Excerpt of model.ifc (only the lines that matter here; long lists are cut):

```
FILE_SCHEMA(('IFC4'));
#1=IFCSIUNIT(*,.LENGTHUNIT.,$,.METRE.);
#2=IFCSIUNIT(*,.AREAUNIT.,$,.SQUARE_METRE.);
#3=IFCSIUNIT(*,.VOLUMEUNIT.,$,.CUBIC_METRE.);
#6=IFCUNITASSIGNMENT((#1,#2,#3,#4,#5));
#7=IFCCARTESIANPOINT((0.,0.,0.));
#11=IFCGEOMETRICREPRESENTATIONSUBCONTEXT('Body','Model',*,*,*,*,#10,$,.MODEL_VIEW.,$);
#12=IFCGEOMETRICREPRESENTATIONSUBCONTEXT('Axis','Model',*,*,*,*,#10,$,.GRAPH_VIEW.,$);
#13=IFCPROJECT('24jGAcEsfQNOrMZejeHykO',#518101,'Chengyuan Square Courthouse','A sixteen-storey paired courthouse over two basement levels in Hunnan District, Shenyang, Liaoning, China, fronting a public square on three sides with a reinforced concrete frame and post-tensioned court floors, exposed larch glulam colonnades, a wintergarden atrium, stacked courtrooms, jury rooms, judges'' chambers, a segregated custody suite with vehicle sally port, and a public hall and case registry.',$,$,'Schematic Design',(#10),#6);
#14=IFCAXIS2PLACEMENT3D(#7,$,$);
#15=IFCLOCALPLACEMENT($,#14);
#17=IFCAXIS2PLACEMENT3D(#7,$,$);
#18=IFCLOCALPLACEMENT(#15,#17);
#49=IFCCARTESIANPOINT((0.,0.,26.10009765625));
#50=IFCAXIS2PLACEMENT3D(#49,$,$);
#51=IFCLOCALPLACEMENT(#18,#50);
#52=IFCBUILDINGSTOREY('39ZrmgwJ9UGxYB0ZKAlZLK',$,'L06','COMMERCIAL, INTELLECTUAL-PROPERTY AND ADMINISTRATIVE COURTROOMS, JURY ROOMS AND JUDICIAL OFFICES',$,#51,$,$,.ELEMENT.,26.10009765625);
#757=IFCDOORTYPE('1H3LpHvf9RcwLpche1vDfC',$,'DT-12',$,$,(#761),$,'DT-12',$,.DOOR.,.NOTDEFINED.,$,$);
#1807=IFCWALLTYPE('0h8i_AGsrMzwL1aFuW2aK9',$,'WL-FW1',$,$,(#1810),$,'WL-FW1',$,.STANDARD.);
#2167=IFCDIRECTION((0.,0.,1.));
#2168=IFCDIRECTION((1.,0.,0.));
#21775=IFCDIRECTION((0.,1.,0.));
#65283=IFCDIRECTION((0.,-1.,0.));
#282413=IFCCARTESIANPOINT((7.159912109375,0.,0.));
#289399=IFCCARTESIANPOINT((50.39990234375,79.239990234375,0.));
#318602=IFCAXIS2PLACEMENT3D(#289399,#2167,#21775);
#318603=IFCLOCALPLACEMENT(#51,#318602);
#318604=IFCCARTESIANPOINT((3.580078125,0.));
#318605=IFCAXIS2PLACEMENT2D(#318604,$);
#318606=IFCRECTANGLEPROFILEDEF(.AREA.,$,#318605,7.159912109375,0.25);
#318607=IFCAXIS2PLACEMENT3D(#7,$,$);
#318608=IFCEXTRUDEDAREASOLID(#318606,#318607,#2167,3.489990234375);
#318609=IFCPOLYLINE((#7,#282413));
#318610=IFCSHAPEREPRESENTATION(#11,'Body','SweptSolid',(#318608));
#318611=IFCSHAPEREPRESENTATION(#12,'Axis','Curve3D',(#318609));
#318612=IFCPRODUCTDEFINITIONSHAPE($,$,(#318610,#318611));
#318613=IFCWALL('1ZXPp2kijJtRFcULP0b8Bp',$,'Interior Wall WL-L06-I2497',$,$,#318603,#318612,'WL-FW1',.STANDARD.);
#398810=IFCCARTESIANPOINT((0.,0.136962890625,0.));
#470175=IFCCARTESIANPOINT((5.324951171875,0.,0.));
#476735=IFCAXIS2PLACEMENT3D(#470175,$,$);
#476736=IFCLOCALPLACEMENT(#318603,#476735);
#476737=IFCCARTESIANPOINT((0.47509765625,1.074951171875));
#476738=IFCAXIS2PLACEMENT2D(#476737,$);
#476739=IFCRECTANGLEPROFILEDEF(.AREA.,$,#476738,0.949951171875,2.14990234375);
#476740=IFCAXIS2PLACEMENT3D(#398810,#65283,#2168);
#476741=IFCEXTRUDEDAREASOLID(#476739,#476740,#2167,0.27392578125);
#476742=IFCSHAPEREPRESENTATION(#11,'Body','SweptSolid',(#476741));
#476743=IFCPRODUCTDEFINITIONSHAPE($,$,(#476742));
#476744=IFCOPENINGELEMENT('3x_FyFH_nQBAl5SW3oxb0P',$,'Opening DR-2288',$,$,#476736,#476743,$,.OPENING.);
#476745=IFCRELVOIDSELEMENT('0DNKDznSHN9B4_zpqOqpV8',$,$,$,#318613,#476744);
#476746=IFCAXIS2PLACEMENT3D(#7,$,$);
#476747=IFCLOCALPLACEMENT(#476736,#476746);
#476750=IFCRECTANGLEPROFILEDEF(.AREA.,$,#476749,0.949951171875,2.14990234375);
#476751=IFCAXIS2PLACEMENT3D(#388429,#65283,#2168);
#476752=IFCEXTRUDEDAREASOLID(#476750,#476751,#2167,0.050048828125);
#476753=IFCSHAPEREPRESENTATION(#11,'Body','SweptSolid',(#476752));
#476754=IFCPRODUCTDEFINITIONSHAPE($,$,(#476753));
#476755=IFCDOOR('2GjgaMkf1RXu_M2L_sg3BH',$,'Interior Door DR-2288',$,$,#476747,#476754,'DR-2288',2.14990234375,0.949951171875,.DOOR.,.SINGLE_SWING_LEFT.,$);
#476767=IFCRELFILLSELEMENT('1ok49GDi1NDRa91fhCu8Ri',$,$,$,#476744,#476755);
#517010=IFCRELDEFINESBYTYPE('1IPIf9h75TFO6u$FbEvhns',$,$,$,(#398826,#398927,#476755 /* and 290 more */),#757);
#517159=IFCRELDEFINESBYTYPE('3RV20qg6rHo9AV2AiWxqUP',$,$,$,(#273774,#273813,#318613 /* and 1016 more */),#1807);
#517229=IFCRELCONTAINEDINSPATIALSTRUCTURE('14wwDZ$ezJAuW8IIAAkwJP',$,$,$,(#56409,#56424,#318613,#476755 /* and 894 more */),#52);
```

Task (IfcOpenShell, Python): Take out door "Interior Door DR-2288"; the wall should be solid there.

```python
import ifcopenshell
import ifcopenshell.api.feature
import ifcopenshell.api.root
import ifcopenshell.geom
import ifcopenshell.util.shape

model = ifcopenshell.open("model.ifc")
settings = ifcopenshell.geom.settings()


def volume(element):
    """Net volume in cubic metres, openings subtracted."""
    shape = ifcopenshell.geom.create_shape(settings, element)
    return ifcopenshell.util.shape.get_volume(shape.geometry)


door = model.by_id(476755)
opening = door.FillsVoids[0].RelatingOpeningElement
wall = opening.VoidsElements[0].RelatingBuildingElement
before = volume(wall)

ifcopenshell.api.root.remove_product(model, product=door)
ifcopenshell.api.feature.remove_feature(model, feature=opening)

after = volume(wall)

print(f"wall volume {before:.3f} -> {after:.3f} m3")

model.write("model_v2.ifc")
```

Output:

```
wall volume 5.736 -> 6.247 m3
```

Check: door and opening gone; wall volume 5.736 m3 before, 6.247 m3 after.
